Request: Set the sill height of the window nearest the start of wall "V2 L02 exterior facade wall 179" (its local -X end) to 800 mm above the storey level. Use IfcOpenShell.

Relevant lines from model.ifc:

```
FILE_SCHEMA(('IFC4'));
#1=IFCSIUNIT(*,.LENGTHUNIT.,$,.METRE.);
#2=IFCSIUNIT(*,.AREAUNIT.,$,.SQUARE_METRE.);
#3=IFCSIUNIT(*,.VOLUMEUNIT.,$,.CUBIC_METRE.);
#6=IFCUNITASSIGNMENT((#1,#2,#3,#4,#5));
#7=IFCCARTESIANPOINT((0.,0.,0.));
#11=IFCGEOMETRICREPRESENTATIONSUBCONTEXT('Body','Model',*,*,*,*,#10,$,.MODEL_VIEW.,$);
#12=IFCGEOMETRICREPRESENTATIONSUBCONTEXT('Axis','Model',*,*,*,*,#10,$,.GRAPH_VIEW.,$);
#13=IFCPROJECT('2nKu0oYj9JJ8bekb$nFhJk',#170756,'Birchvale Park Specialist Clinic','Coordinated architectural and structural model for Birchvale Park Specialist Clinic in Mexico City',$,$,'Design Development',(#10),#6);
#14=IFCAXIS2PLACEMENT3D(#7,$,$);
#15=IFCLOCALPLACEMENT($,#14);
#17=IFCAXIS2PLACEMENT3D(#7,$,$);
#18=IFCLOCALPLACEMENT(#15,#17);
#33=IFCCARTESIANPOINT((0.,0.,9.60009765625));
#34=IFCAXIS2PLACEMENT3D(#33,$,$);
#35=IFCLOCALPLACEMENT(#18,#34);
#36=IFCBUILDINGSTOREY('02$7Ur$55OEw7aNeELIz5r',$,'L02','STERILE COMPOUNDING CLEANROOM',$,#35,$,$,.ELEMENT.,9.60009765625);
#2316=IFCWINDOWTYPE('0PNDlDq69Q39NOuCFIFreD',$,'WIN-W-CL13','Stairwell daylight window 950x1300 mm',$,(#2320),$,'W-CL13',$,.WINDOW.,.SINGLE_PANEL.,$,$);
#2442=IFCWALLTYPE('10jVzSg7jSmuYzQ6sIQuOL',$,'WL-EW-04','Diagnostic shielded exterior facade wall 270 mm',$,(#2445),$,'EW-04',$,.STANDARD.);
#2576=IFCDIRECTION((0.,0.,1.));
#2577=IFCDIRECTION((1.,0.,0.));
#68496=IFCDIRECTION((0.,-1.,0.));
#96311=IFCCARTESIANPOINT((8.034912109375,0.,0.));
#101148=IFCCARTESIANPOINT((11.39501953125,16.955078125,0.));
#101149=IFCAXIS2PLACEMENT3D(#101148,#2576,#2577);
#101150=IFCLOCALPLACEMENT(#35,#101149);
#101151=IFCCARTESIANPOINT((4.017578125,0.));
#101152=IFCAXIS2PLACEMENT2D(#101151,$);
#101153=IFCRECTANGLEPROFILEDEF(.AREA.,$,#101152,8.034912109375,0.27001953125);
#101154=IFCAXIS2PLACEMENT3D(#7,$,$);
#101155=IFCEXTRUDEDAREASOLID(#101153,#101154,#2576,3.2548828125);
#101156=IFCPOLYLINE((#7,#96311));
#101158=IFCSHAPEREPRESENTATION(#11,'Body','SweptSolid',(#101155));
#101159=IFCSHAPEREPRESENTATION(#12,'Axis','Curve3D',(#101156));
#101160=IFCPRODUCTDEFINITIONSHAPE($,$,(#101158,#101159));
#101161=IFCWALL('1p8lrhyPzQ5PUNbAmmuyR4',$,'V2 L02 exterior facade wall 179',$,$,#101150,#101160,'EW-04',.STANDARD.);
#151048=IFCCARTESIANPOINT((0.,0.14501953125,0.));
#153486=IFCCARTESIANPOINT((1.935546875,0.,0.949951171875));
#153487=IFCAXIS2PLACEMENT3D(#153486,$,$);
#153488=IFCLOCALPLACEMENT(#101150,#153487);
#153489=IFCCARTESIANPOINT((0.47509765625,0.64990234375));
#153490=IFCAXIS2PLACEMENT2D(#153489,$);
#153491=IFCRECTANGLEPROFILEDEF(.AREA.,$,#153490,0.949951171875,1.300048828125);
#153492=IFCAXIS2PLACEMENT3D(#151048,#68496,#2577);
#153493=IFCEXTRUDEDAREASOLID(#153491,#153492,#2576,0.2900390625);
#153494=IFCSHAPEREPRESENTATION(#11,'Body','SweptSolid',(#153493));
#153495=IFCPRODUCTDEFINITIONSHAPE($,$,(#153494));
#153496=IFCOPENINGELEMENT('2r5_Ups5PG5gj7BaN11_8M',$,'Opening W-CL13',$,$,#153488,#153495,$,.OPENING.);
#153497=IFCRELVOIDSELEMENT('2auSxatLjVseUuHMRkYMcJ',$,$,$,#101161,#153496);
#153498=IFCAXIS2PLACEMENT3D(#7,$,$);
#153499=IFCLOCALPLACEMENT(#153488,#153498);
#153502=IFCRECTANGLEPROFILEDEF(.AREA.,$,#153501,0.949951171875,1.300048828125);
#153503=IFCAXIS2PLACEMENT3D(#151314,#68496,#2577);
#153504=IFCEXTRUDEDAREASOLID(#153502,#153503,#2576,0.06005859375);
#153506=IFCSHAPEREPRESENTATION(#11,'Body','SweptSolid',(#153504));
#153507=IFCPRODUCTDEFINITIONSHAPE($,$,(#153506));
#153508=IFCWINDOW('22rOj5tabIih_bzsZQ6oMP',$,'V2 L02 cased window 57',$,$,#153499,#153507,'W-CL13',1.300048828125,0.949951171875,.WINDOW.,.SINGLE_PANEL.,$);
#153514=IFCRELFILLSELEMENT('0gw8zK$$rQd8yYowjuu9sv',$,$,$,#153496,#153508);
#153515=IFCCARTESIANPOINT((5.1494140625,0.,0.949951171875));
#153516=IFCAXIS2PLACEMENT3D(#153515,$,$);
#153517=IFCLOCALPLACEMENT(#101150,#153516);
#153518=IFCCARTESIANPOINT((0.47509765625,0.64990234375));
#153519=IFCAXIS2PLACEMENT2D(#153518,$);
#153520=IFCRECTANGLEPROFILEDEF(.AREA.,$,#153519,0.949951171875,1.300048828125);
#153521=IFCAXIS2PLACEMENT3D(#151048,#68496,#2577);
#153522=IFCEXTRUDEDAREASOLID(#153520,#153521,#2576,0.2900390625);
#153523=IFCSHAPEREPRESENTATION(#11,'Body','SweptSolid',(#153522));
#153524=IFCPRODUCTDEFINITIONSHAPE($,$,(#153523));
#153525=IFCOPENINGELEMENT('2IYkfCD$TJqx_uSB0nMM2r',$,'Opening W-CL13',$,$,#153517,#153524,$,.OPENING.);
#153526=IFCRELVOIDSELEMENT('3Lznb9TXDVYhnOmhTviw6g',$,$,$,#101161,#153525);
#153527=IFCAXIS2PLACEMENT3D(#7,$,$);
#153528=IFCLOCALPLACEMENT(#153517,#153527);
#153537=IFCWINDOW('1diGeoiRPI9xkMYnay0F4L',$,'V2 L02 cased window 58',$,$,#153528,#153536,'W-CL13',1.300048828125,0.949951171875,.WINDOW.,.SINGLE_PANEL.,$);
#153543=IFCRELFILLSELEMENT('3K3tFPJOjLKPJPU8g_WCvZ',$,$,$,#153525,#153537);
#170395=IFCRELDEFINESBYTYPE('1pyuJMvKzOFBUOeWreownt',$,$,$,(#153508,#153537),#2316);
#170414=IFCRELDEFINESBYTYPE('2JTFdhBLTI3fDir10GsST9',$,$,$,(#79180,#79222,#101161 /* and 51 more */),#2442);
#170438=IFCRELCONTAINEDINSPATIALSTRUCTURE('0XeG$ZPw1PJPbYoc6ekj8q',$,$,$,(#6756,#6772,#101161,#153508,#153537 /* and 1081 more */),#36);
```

```python
import numpy as np
import ifcopenshell
import ifcopenshell.api.geometry
import ifcopenshell.geom
import ifcopenshell.util.element
import ifcopenshell.util.placement
import ifcopenshell.util.shape
import ifcopenshell.util.unit

model = ifcopenshell.open("model.ifc")
unit_scale = ifcopenshell.util.unit.calculate_unit_scale(model)

window = model.by_id(153508)
opening = window.FillsVoids[0].RelatingOpeningElement
storey = ifcopenshell.util.element.get_container(window, ifc_class="IfcBuildingStorey")
level = ifcopenshell.util.placement.get_local_placement(storey.ObjectPlacement)[2, 3]

# The opening's origin need not be at the sill, so measure its lowest point.
shape = ifcopenshell.geom.create_shape(ifcopenshell.geom.settings(), opening)
bottom = ifcopenshell.util.shape.get_shape_bottom_elevation(shape, shape.geometry) / unit_scale
dz = level + 0.8 / unit_scale - bottom

shift = np.array([0.0, 0.0, dz])
# The window is placed relative to its opening, so it follows when the opening moves.
matrix = ifcopenshell.util.placement.get_local_placement(opening.ObjectPlacement)
matrix[:3, 3] += shift
ifcopenshell.api.geometry.edit_object_placement(
    model, product=opening, matrix=matrix, is_si=False, should_transform_children=True
)

print(f"moved by {dz * unit_scale:+.3f} m")

model.write("model_v2.ifc")
```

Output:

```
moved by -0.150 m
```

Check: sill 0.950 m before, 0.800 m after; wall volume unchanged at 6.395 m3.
